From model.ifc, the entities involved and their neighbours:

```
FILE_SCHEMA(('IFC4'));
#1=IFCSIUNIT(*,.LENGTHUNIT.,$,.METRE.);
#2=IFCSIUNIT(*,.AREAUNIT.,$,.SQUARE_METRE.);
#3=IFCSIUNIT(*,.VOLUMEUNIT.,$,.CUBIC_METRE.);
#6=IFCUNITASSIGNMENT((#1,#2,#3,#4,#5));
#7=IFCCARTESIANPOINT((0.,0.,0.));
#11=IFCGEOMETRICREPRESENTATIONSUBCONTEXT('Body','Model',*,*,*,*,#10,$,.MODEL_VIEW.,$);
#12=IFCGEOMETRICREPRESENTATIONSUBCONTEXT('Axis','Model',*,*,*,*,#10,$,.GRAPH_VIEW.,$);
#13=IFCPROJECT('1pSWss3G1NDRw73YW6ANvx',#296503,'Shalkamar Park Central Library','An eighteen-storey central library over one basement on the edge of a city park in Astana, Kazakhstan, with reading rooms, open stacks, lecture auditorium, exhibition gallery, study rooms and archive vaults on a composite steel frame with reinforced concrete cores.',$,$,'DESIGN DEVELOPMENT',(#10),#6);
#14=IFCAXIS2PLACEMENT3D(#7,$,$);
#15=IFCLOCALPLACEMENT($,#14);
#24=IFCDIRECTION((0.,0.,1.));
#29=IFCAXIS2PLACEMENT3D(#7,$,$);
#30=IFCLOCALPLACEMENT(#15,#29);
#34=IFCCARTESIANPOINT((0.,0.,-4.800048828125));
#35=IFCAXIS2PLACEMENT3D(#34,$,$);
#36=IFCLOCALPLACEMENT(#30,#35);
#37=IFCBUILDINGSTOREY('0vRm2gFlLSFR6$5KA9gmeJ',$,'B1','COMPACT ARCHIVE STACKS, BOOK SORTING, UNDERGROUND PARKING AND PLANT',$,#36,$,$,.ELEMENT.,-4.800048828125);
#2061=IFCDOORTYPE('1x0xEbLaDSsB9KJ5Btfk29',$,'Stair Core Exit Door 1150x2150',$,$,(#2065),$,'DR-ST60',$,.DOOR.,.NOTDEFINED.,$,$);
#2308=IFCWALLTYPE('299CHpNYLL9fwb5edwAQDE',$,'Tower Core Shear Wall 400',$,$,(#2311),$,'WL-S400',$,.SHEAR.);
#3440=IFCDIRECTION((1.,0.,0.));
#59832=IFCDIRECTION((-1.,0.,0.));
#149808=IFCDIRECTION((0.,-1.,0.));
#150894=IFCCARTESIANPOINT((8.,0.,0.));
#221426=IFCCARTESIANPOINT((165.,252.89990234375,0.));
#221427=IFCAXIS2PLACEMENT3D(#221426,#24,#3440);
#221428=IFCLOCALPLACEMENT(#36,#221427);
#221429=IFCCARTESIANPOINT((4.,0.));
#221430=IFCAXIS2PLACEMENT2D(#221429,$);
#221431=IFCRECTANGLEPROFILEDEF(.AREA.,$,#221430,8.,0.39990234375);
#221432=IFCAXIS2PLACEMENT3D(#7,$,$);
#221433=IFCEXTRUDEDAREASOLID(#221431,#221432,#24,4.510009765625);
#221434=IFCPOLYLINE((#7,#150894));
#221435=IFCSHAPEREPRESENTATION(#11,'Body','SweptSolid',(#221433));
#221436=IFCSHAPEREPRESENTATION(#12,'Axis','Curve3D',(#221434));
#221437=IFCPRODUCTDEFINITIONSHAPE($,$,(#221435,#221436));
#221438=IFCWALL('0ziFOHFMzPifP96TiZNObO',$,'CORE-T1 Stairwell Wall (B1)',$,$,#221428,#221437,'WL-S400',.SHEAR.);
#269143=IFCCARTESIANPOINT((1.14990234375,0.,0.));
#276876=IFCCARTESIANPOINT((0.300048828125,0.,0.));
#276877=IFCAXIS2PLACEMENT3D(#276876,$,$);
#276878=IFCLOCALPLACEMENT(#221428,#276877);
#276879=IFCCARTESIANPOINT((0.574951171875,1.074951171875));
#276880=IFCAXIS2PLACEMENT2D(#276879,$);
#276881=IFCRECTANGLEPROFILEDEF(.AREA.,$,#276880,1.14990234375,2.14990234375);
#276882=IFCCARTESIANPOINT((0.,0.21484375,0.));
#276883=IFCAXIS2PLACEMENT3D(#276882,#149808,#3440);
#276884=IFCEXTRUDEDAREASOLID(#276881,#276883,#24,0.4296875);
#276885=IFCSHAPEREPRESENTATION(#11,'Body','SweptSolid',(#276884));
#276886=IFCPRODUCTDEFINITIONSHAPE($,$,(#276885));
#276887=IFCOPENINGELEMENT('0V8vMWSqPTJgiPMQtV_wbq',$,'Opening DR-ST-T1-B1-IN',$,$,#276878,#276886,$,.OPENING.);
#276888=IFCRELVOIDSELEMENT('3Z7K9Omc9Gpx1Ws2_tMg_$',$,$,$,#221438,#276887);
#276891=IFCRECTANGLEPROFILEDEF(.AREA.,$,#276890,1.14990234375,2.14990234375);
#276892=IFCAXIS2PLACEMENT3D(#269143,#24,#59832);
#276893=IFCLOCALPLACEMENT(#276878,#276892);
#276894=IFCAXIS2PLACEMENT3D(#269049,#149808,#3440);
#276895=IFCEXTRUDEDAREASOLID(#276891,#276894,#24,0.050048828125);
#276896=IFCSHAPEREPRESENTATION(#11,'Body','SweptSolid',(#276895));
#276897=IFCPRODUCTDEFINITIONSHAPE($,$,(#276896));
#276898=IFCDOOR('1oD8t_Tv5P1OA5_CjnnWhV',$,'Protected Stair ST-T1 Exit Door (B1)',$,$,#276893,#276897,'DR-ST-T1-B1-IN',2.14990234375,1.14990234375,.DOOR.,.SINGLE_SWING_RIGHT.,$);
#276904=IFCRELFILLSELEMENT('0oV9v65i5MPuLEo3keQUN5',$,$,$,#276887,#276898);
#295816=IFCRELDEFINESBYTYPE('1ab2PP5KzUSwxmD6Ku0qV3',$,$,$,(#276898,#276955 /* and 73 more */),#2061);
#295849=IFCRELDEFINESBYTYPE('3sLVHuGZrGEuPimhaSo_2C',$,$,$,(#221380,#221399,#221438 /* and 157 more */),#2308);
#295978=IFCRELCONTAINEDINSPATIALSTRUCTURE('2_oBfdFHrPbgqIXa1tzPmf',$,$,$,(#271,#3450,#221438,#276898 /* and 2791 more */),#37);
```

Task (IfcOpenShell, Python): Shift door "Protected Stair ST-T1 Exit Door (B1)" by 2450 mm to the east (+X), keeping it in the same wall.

```python
import ifcopenshell
import ifcopenshell.api.geometry
import ifcopenshell.util.placement
import ifcopenshell.util.unit

model = ifcopenshell.open("model.ifc")
unit_scale = ifcopenshell.util.unit.calculate_unit_scale(model)

door = model.by_guid("1oD8t_Tv5P1OA5_CjnnWhV")
opening = door.FillsVoids[0].RelatingOpeningElement
wall = opening.VoidsElements[0].RelatingBuildingElement

wall_matrix = ifcopenshell.util.placement.get_local_placement(wall.ObjectPlacement)
shift = wall_matrix[:3, 0] * 2.45 / unit_scale
before = ifcopenshell.util.placement.get_local_placement(door.ObjectPlacement)[:3, 3].copy()

# The door is placed relative to its opening, so it follows when the opening moves.
matrix = ifcopenshell.util.placement.get_local_placement(opening.ObjectPlacement)
matrix[:3, 3] += shift
ifcopenshell.api.geometry.edit_object_placement(
    model, product=opening, matrix=matrix, is_si=False, should_transform_children=True
)

after = ifcopenshell.util.placement.get_local_placement(door.ObjectPlacement)[:3, 3]
print("door moved by", (after - before).round(3) + 0.0)

model.write("model_v2.ifc")
```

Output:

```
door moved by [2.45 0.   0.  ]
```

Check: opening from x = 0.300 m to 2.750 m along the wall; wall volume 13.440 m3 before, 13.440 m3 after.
